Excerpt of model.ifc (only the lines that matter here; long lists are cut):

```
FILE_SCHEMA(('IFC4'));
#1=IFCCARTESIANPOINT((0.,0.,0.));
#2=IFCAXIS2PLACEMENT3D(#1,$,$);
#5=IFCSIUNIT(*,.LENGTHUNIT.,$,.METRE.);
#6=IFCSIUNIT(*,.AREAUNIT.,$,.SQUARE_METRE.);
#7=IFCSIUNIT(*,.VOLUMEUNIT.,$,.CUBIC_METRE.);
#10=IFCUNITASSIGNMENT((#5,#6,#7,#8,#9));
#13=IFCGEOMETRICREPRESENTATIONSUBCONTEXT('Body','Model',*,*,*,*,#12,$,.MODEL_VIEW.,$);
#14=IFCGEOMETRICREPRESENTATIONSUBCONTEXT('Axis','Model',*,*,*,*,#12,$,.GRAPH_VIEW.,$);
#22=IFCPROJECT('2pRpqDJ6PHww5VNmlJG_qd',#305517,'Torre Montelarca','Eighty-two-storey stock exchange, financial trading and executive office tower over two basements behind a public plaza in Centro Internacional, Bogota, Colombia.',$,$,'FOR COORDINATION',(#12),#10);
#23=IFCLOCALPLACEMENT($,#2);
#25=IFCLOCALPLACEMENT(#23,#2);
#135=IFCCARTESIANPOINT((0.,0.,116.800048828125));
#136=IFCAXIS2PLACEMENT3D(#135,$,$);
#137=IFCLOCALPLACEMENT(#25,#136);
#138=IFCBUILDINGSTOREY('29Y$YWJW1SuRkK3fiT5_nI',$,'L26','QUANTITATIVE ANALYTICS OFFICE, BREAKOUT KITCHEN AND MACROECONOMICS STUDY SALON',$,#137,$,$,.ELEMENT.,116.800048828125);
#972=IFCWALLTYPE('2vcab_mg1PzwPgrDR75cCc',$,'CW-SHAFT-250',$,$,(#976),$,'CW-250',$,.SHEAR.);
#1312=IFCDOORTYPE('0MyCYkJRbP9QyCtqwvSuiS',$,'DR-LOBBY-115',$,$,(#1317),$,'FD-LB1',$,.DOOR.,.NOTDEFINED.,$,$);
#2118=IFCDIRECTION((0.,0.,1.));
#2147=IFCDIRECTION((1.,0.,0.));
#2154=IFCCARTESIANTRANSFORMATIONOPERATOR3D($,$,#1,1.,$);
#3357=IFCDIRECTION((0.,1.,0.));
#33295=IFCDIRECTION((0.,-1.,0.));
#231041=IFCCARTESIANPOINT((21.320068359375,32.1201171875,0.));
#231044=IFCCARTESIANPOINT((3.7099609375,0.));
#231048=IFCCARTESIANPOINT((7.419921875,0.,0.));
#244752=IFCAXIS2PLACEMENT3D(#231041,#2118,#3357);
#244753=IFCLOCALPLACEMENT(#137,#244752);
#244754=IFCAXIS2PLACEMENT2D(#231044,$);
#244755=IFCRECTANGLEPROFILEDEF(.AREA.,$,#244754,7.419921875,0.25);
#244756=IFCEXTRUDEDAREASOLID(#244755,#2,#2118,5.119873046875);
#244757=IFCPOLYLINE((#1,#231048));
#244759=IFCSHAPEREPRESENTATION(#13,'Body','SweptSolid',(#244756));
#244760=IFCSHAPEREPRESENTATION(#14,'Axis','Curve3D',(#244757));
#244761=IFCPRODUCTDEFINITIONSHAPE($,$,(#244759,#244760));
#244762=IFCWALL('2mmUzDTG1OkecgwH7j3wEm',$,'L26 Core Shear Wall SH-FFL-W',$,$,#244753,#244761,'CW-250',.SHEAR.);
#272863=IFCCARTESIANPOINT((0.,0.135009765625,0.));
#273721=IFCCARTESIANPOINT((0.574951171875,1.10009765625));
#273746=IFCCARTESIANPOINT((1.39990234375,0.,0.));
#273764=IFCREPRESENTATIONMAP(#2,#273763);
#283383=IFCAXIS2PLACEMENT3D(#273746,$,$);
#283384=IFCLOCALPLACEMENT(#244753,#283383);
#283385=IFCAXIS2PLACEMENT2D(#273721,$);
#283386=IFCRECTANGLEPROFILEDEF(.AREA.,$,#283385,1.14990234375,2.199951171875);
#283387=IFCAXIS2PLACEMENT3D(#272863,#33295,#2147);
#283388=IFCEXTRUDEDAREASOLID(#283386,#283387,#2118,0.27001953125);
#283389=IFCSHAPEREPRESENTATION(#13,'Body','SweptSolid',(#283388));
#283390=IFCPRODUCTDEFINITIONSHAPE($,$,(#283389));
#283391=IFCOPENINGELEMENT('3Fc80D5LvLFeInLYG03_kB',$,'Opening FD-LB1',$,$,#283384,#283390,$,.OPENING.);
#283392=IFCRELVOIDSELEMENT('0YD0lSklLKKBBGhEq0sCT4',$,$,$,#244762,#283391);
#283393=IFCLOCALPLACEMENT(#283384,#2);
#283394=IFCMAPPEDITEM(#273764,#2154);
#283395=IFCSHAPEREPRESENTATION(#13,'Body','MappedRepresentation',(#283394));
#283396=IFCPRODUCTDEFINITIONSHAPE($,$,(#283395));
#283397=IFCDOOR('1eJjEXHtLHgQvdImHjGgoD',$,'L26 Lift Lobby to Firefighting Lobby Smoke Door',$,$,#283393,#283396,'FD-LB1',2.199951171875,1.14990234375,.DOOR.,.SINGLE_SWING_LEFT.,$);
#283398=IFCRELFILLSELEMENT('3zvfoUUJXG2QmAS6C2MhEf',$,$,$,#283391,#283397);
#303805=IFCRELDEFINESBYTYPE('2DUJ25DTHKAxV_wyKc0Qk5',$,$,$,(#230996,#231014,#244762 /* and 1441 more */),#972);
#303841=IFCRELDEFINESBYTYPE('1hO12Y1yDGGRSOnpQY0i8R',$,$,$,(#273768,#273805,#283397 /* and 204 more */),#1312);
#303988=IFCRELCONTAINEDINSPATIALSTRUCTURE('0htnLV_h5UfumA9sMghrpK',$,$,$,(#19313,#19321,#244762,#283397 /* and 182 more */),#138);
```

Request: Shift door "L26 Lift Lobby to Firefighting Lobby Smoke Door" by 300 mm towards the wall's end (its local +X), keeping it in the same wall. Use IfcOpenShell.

```python
import ifcopenshell
import ifcopenshell.api.geometry
import ifcopenshell.util.placement
import ifcopenshell.util.unit

model = ifcopenshell.open("model.ifc")
unit_scale = ifcopenshell.util.unit.calculate_unit_scale(model)

door = model.by_guid("1eJjEXHtLHgQvdImHjGgoD")
opening = door.FillsVoids[0].RelatingOpeningElement
wall = opening.VoidsElements[0].RelatingBuildingElement

wall_matrix = ifcopenshell.util.placement.get_local_placement(wall.ObjectPlacement)
shift = wall_matrix[:3, 0] * 0.3 / unit_scale
before = ifcopenshell.util.placement.get_local_placement(door.ObjectPlacement)[:3, 3].copy()

# The door is placed relative to its opening, so it follows when the opening moves.
matrix = ifcopenshell.util.placement.get_local_placement(opening.ObjectPlacement)
matrix[:3, 3] += shift
ifcopenshell.api.geometry.edit_object_placement(
    model, product=opening, matrix=matrix, is_si=False, should_transform_children=True
)

after = ifcopenshell.util.placement.get_local_placement(door.ObjectPlacement)[:3, 3]
print("door moved by", (after - before).round(3) + 0.0)

model.write("model_v2.ifc")
```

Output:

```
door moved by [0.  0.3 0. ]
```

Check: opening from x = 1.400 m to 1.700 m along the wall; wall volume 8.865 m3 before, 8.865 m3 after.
